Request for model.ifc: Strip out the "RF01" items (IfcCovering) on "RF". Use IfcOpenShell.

First a look at what the model holds.

```python
import ifcopenshell
import ifcopenshell.util.element

model = ifcopenshell.open("model.ifc")
print(model.schema)
storey = next(s for s in model.by_type("IfcBuildingStorey") if s.Name == "RF")
coverings = [e for e in ifcopenshell.util.element.get_decomposition(storey) if e.is_a("IfcCovering")]
seen = {}
for e in coverings:
    element_type = ifcopenshell.util.element.get_type(e)
    name = element_type.Name if element_type not in (None, e) else None
    seen[name] = seen.get(name, 0) + 1
for name, count in sorted(seen.items(), key=str):
    print(count, "x", name)
```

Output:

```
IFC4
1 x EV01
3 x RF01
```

```python
import ifcopenshell
import ifcopenshell.api.root
import ifcopenshell.util.element

model = ifcopenshell.open("model.ifc")

storey = next(s for s in model.by_type("IfcBuildingStorey") if s.Name == "RF")
coverings = [e for e in ifcopenshell.util.element.get_decomposition(storey) if e.is_a("IfcCovering")]
targets = [e for e in coverings if (t := ifcopenshell.util.element.get_type(e)) not in (None, e) and t.Name == "RF01"]

for e in targets:
    ifcopenshell.api.root.remove_product(model, product=e)
print(len(targets), "removed")

model.write("model_v2.ifc")
```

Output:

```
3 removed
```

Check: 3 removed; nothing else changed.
